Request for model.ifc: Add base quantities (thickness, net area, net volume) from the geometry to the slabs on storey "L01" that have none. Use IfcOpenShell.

First a look at what the model holds.

```python
import ifcopenshell
import ifcopenshell.util.element
import ifcopenshell.util.unit

model = ifcopenshell.open("model.ifc")
print(model.schema)
for unit_type in ("LENGTHUNIT", "AREAUNIT", "VOLUMEUNIT"):
    print(unit_type, ifcopenshell.util.unit.calculate_unit_scale(model, unit_type))
storey = next(s for s in model.by_type("IfcBuildingStorey") if s.Name == "L01")
slabs = [e for e in ifcopenshell.util.element.get_decomposition(storey) if e.is_a("IfcSlab")]
for e in sorted(slabs, key=lambda e: e.id()):
    print(e.id(), e.is_a(), e.Name, list(ifcopenshell.util.element.get_psets(e, qtos_only=True)), sep=" | ")
```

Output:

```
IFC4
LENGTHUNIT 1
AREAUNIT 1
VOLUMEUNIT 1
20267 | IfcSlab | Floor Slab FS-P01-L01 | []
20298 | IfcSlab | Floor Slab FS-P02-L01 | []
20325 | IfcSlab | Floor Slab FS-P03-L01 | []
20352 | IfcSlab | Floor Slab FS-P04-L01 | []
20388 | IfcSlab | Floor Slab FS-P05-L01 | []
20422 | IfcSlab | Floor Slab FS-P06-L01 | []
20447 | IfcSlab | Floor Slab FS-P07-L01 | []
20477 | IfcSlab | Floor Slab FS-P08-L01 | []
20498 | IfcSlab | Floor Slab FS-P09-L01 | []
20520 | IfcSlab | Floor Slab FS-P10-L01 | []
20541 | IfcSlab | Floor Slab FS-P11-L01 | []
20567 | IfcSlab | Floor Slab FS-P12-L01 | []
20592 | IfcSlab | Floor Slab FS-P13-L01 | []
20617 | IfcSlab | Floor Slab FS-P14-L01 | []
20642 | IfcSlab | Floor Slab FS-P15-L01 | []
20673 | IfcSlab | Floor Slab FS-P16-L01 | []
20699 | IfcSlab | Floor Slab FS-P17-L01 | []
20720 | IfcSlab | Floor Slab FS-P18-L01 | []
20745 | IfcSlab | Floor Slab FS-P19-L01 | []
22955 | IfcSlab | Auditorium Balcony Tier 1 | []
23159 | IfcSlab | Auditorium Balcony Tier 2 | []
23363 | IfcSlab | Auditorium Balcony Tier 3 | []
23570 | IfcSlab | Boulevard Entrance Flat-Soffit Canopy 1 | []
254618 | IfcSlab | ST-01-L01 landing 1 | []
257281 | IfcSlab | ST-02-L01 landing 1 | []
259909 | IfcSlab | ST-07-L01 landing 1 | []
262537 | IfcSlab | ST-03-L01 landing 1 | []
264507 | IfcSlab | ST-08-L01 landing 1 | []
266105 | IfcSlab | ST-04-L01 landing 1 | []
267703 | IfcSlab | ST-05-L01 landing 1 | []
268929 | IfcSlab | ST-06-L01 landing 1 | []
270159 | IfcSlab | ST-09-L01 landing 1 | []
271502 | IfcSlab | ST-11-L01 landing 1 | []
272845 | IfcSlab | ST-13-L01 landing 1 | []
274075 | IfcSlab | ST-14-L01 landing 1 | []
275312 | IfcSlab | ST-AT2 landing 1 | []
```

```python
import ifcopenshell
import ifcopenshell.api.pset
import ifcopenshell.geom
import ifcopenshell.util.element
import ifcopenshell.util.shape
import ifcopenshell.util.unit

model = ifcopenshell.open("model.ifc")
unit_scale = ifcopenshell.util.unit.calculate_unit_scale(model)
area_scale = ifcopenshell.util.unit.calculate_unit_scale(model, "AREAUNIT")
volume_scale = ifcopenshell.util.unit.calculate_unit_scale(model, "VOLUMEUNIT")
settings = ifcopenshell.geom.settings()

storey = next(s for s in model.by_type("IfcBuildingStorey") if s.Name == "L01")
slabs = [e for e in ifcopenshell.util.element.get_decomposition(storey) if e.is_a("IfcSlab")]

for e in sorted(slabs, key=lambda e: e.id()):
    if ifcopenshell.util.element.get_psets(e, qtos_only=True, should_inherit=False):
        continue
    # Geometry comes back in metres, in the element's own axes.
    shape = ifcopenshell.geom.create_shape(settings, e)
    values = {
        "Width": ifcopenshell.util.shape.get_z(shape.geometry) / unit_scale,
        "NetArea": ifcopenshell.util.shape.get_footprint_area(shape.geometry) / area_scale,
        "NetVolume": ifcopenshell.util.shape.get_volume(shape.geometry) / volume_scale,
    }
    qto = ifcopenshell.api.pset.add_qto(model, product=e, name="Qto_SlabBaseQuantities")
    ifcopenshell.api.pset.edit_qto(model, qto=qto, properties=values)
    print(e.id(), {k: round(v, 3) for k, v in values.items()})

model.write("model_edited.ifc")
```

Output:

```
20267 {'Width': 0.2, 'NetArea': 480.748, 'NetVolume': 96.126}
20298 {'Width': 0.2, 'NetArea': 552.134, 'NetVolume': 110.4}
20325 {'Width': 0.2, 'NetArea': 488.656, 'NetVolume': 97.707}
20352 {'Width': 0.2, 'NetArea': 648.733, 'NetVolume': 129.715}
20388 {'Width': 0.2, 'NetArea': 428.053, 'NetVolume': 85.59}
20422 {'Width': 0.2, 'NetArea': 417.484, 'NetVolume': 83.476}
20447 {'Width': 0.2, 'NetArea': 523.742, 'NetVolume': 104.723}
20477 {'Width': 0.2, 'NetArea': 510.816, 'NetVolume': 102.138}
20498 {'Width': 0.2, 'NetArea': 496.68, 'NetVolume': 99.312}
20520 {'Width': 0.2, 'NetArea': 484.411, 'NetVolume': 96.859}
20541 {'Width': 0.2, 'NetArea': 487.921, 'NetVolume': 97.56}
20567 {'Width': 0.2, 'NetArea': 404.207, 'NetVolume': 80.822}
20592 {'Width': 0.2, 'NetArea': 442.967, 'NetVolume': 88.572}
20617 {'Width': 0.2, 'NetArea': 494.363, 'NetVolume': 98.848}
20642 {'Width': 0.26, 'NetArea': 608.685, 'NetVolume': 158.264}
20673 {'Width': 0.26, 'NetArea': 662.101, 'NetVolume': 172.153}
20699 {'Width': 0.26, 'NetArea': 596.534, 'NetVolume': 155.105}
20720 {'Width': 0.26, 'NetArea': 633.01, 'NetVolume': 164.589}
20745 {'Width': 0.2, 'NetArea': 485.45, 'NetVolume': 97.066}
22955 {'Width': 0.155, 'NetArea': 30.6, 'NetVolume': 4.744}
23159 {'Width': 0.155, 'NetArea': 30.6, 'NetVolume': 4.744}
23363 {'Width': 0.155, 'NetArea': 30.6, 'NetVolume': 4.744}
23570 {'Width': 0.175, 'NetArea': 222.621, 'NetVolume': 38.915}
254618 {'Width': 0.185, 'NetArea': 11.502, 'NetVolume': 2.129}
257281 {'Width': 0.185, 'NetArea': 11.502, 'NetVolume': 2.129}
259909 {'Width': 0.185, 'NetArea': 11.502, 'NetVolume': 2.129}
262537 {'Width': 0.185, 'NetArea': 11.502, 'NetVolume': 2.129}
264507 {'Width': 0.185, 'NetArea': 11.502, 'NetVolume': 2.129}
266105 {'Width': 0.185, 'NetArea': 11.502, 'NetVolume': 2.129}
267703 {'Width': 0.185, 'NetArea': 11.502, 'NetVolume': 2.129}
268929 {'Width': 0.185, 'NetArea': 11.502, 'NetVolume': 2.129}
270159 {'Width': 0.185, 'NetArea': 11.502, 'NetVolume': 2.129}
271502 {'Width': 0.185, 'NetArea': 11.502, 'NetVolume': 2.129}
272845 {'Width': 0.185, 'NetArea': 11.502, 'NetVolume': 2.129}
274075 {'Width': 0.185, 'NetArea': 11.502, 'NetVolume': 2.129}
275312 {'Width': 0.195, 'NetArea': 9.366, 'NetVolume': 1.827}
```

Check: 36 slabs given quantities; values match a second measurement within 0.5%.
